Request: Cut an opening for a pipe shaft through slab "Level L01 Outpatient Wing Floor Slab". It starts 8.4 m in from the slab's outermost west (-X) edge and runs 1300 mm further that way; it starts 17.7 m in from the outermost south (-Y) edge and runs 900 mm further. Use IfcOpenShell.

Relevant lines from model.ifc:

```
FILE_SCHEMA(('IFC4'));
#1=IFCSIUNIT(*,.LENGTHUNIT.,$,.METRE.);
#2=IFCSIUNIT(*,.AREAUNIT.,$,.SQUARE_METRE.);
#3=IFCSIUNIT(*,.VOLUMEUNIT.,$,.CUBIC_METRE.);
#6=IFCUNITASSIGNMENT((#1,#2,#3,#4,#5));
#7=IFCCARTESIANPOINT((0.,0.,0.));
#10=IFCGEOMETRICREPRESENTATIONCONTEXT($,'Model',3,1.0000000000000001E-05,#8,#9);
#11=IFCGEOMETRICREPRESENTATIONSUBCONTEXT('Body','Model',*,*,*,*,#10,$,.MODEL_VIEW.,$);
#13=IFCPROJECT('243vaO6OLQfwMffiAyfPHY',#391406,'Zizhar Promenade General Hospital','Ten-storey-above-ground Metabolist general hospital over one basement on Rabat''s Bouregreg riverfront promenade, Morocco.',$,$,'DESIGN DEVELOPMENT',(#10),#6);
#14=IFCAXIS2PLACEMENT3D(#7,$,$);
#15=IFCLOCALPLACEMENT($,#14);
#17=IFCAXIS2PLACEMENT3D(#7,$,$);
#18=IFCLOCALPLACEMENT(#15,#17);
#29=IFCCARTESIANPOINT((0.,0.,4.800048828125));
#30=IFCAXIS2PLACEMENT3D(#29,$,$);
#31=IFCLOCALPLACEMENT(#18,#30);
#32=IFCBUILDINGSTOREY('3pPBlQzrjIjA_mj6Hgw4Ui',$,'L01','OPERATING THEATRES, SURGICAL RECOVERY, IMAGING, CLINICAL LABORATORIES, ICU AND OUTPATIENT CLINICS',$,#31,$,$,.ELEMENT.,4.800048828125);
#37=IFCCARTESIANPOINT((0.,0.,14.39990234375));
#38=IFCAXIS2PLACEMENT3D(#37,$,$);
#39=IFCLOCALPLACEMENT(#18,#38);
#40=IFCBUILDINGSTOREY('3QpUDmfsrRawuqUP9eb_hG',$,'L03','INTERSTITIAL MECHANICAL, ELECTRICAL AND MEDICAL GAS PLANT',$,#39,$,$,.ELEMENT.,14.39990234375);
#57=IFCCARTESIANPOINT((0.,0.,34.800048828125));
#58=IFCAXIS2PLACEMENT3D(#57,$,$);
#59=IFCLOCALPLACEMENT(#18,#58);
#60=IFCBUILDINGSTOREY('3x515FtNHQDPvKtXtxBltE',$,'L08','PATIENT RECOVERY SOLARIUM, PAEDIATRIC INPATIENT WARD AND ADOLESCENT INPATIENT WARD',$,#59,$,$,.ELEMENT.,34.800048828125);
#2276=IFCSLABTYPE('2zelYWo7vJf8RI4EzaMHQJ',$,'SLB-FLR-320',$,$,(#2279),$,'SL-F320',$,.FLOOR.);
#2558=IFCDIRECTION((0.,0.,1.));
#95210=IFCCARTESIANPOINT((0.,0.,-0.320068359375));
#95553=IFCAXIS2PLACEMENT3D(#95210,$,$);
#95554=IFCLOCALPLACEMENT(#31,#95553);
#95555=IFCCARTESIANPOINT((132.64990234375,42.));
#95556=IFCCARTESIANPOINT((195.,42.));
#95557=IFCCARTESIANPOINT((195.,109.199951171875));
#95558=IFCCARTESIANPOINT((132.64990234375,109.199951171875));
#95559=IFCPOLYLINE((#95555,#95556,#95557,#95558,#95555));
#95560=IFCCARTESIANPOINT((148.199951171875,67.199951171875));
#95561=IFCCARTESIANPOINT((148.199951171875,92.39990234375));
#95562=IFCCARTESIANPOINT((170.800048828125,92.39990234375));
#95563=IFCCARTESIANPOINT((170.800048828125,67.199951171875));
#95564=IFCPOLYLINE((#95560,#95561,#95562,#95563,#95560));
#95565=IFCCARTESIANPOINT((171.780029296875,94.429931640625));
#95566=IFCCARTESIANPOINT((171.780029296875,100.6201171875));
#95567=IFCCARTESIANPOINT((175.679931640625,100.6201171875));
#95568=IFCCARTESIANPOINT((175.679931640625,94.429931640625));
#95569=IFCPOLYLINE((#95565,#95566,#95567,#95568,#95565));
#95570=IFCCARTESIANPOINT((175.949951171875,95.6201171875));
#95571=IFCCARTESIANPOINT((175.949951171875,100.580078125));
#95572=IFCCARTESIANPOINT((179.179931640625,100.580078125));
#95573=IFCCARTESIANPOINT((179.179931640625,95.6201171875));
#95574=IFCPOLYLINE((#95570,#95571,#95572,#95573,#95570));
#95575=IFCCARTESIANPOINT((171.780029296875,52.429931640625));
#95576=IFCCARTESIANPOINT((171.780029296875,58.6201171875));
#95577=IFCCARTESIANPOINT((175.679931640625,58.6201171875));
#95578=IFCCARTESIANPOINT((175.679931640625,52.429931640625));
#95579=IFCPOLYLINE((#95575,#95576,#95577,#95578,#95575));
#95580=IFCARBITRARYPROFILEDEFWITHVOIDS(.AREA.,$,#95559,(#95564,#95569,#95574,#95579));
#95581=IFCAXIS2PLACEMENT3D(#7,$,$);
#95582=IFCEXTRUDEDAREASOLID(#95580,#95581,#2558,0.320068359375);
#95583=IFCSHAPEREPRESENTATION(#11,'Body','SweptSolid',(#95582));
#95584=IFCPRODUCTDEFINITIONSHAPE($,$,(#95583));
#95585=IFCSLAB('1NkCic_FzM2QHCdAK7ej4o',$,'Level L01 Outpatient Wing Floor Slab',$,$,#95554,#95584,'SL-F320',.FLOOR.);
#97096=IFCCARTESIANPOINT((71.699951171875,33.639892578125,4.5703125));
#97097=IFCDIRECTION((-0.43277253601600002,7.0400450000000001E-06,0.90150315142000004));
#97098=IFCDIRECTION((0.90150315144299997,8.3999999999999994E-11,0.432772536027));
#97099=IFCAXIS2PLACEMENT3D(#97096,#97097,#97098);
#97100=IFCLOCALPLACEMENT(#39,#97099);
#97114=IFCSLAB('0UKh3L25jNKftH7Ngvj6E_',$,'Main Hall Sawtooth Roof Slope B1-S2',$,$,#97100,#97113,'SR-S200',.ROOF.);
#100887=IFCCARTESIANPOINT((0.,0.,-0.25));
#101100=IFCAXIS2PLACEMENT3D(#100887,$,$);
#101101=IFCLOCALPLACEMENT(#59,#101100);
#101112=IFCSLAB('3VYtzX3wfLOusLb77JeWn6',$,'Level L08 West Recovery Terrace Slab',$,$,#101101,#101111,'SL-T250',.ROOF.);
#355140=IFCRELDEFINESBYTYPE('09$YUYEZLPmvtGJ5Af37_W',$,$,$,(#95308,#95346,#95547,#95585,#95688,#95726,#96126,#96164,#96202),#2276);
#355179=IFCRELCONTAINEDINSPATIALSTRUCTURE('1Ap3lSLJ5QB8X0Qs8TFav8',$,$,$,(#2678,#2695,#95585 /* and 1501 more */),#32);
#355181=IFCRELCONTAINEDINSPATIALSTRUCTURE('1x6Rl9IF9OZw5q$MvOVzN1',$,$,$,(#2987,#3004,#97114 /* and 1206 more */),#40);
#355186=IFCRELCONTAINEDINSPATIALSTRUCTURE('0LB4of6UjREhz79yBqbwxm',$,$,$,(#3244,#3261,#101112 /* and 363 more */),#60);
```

```python
import numpy as np
import ifcopenshell
import ifcopenshell.api.feature
import ifcopenshell.api.geometry
import ifcopenshell.api.root
import ifcopenshell.geom
import ifcopenshell.util.placement
import ifcopenshell.util.representation
import ifcopenshell.util.shape
import ifcopenshell.util.unit

model = ifcopenshell.open("model.ifc")
unit_scale = ifcopenshell.util.unit.calculate_unit_scale(model)
settings = ifcopenshell.geom.settings()


def volume(element):
    """Net volume in cubic metres, openings subtracted."""
    shape = ifcopenshell.geom.create_shape(settings, element)
    return ifcopenshell.util.shape.get_volume(shape.geometry)


slab = model.by_guid("1NkCic_FzM2QHCdAK7ej4o")
before = volume(slab)

# Extent in the slab's own axes, in metres. The edges named are its -X and -Y sides.
slab_shape = ifcopenshell.geom.create_shape(settings, slab)
vertices = ifcopenshell.util.shape.get_vertices(slab_shape.geometry)
x_min, y_min, bottom = vertices.min(axis=0)
top = vertices[:, 2].max()

opening = ifcopenshell.api.root.create_entity(model, ifc_class="IfcOpeningElement", name="Pipe shaft opening", predefined_type="OPENING")
context = ifcopenshell.util.representation.get_context(model, "Model", "Body", "MODEL_VIEW")
width, depth = 1.3, 0.9
outline = [(0.0, 0.0), (width, 0.0), (width, depth), (0.0, depth), (0.0, 0.0)]
# Overshoot both faces by 50 mm so the cut is clean.
shape = ifcopenshell.api.geometry.add_slab_representation(
    model, context=context, depth=top - bottom + 0.1, polyline=outline
)
ifcopenshell.api.geometry.assign_representation(model, product=opening, representation=shape)

matrix = ifcopenshell.util.placement.get_local_placement(slab.ObjectPlacement)
matrix[:, 3] = matrix @ np.append(np.array([x_min + 8.4, y_min + 17.7, bottom - 0.05]) / unit_scale, 1.0)
ifcopenshell.api.geometry.edit_object_placement(model, product=opening, matrix=matrix, is_si=False)
ifcopenshell.api.feature.add_feature(model, feature=opening, element=slab)

after = volume(slab)

print(f"slab volume {before:.3f} -> {after:.3f} m3")

model.write("model_rev.ifc")
```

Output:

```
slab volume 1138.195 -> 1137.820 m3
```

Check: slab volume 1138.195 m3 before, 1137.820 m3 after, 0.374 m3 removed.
